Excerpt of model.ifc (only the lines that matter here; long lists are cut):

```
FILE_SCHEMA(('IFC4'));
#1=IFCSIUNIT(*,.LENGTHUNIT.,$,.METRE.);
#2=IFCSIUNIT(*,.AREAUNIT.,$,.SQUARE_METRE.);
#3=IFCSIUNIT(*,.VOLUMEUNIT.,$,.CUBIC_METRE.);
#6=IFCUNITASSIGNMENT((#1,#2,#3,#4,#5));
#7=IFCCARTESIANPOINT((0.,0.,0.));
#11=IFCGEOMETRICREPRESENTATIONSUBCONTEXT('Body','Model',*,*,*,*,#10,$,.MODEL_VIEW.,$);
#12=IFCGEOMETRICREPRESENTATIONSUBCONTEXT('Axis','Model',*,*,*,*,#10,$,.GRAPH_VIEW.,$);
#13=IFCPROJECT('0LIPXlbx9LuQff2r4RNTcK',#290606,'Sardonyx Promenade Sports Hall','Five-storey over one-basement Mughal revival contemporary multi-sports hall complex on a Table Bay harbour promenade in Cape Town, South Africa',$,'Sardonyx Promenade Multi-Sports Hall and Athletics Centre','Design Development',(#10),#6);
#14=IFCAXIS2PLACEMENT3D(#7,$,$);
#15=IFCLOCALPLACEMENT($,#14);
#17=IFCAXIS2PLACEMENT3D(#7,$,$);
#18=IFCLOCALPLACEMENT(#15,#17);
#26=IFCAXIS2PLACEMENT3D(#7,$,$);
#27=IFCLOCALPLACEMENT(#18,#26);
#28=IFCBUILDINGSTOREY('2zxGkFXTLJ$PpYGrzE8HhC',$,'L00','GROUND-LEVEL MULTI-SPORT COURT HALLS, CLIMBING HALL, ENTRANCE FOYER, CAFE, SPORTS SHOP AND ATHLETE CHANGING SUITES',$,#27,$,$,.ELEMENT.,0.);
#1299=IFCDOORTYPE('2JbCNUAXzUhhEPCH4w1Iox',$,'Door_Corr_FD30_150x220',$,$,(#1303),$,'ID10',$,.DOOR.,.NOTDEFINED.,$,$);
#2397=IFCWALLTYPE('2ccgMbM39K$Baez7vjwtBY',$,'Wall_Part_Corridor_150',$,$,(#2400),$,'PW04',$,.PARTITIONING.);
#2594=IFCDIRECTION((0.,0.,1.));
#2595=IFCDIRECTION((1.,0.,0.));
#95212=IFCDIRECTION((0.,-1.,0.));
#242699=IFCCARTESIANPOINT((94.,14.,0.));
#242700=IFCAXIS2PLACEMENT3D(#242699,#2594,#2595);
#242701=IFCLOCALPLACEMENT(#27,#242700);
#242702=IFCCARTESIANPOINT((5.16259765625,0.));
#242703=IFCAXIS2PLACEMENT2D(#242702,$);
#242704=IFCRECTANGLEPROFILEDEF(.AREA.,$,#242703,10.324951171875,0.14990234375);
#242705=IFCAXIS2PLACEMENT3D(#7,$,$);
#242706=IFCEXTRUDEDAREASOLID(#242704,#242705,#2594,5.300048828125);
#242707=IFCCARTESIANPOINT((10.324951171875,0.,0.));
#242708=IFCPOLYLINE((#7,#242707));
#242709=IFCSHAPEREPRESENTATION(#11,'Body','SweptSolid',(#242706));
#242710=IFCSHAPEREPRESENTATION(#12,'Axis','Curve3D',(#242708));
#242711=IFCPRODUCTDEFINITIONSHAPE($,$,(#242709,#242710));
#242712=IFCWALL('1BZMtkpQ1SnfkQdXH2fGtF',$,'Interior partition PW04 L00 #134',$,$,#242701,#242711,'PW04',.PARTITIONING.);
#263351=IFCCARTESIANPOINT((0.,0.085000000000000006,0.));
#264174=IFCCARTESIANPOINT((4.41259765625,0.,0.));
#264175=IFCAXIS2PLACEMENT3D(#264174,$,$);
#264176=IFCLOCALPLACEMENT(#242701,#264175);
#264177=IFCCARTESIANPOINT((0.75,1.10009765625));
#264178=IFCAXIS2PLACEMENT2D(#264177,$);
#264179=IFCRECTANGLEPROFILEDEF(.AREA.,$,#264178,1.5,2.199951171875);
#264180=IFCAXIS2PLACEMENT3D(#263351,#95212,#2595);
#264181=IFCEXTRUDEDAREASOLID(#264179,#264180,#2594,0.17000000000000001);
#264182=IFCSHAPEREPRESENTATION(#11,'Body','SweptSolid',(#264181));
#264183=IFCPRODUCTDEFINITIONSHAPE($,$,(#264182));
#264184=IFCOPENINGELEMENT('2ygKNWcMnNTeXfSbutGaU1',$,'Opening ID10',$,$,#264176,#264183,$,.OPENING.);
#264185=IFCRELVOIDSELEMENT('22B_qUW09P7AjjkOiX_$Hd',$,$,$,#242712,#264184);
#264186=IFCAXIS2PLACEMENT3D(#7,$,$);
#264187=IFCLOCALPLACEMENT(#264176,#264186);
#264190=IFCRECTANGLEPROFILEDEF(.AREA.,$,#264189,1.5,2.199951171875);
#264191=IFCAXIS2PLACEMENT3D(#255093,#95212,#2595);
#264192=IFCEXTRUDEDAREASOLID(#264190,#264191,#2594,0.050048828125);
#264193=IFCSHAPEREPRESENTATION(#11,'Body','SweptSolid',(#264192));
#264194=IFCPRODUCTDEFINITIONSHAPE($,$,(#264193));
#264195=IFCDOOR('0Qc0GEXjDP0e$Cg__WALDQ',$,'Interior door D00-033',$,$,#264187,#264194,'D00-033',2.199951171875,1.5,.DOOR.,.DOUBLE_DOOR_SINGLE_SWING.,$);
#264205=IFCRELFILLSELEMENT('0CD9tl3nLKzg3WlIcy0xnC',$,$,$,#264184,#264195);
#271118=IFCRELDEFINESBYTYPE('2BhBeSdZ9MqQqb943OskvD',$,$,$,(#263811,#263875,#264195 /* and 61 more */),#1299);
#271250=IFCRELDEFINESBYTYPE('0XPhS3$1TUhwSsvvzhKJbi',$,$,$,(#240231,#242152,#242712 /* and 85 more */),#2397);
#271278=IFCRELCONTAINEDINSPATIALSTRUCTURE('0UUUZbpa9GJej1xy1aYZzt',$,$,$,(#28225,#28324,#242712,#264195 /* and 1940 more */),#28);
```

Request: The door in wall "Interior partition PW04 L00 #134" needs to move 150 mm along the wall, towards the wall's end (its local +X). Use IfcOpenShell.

```python
import ifcopenshell
import ifcopenshell.api.geometry
import ifcopenshell.util.placement

model = ifcopenshell.open("model.ifc")

door = model.by_id(264195)
opening = door.FillsVoids[0].RelatingOpeningElement
wall = opening.VoidsElements[0].RelatingBuildingElement

wall_matrix = ifcopenshell.util.placement.get_local_placement(wall.ObjectPlacement)
shift = wall_matrix[:3, 0] * 0.15
before = ifcopenshell.util.placement.get_local_placement(door.ObjectPlacement)[:3, 3].copy()

# The door is placed relative to its opening, so it follows when the opening moves.
matrix = ifcopenshell.util.placement.get_local_placement(opening.ObjectPlacement)
matrix[:3, 3] += shift
ifcopenshell.api.geometry.edit_object_placement(
    model, product=opening, matrix=matrix, is_si=False, should_transform_children=True
)

after = ifcopenshell.util.placement.get_local_placement(door.ObjectPlacement)[:3, 3]
print("door moved by", (after - before).round(3) + 0.0)

model.write("model_v2.ifc")
```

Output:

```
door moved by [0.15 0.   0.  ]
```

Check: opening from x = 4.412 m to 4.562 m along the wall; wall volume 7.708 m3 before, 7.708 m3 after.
